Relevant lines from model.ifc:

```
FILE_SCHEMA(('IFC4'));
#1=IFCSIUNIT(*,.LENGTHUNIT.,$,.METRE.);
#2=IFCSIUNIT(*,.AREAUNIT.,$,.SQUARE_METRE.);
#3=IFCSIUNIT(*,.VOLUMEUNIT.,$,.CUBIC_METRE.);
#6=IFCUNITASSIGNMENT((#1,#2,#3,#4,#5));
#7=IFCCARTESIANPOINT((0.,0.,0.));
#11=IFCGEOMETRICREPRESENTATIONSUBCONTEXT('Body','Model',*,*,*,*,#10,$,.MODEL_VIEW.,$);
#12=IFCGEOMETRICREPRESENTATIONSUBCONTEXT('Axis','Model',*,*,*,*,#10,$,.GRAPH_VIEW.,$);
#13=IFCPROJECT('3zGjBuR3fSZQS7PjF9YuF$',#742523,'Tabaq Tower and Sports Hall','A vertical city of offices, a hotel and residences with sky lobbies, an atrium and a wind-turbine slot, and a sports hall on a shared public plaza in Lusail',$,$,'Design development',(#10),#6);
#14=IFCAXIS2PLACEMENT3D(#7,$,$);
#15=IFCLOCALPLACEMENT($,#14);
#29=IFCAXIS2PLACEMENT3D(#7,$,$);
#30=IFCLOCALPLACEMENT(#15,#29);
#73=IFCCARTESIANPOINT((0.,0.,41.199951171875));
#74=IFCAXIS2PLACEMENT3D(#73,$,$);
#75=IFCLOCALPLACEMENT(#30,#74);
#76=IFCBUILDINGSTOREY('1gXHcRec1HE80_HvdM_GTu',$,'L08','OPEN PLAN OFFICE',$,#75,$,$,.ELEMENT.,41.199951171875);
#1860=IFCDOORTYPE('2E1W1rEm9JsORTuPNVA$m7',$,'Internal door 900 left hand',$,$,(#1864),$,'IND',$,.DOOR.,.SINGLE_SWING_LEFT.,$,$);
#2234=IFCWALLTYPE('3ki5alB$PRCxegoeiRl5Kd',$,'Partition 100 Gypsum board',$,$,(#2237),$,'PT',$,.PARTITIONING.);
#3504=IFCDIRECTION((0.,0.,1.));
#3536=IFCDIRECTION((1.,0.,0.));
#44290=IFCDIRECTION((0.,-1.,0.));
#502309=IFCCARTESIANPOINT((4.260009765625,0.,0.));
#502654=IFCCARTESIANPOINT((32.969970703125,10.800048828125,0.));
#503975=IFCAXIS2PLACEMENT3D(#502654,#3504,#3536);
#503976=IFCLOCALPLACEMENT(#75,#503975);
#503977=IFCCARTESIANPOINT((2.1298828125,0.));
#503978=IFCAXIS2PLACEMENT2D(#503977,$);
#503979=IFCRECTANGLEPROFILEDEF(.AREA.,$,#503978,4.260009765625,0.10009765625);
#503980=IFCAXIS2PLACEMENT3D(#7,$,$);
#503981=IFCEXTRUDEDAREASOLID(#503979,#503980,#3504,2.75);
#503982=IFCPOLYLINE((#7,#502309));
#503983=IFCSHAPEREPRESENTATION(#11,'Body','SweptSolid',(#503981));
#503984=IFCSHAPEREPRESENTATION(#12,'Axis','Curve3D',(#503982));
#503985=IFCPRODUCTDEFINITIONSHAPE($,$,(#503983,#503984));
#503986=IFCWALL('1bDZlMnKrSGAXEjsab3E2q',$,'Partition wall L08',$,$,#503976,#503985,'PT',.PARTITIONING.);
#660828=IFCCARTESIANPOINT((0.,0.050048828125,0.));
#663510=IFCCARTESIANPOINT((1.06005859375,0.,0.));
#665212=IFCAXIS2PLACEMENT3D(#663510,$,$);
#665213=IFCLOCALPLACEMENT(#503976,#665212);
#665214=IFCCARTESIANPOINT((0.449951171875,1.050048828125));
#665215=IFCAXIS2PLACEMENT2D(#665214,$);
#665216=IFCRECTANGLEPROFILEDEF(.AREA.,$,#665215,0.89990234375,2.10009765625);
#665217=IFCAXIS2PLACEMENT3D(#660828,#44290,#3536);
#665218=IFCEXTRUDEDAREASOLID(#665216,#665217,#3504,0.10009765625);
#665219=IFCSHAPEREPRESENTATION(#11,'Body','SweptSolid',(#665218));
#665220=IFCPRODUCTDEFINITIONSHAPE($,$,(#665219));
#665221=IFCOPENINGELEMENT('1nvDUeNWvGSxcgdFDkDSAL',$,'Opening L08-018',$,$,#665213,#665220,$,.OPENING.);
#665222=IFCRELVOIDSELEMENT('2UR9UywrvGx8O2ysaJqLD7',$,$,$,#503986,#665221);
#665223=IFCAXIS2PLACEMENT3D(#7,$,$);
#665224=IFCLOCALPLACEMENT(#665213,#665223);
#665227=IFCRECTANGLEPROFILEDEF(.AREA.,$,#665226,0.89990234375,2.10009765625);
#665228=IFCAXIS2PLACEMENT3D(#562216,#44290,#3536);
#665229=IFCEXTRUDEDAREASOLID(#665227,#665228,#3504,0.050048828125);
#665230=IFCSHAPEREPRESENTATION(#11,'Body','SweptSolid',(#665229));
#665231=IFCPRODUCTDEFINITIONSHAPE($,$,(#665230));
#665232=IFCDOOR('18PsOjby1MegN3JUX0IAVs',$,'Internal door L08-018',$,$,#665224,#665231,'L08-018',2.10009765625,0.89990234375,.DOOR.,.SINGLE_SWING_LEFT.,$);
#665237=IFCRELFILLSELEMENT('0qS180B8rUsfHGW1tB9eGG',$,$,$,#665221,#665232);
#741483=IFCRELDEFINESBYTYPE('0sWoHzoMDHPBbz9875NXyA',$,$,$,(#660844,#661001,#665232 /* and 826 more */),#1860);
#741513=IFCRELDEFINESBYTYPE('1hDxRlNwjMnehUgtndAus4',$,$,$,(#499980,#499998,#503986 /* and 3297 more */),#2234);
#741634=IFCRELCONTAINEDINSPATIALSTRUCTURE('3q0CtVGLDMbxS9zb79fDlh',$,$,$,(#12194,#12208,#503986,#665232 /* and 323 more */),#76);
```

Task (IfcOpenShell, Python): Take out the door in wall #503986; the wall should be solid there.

```python
import ifcopenshell
import ifcopenshell.api.feature
import ifcopenshell.api.root
import ifcopenshell.geom
import ifcopenshell.util.shape

model = ifcopenshell.open("model.ifc")
settings = ifcopenshell.geom.settings()


def volume(element):
    """Net volume in cubic metres, openings subtracted."""
    shape = ifcopenshell.geom.create_shape(settings, element)
    return ifcopenshell.util.shape.get_volume(shape.geometry)


door = model.by_guid("18PsOjby1MegN3JUX0IAVs")
opening = door.FillsVoids[0].RelatingOpeningElement
wall = opening.VoidsElements[0].RelatingBuildingElement
before = volume(wall)

ifcopenshell.api.root.remove_product(model, product=door)
ifcopenshell.api.feature.remove_feature(model, feature=opening)

after = volume(wall)

print(f"wall volume {before:.3f} -> {after:.3f} m3")

model.write("model_updated.ifc")
```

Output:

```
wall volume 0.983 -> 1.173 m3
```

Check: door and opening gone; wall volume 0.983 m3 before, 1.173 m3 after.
